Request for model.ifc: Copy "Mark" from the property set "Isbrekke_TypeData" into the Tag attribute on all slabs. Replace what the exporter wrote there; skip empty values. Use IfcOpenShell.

First a look at what the model holds.

```python
import ifcopenshell
import ifcopenshell.util.element

model = ifcopenshell.open("model.ifc")
print(model.schema)
slabs = model.by_type("IfcSlab")
print(len(slabs), "slabs")
for e in slabs[:8]:
    source = ifcopenshell.util.element.get_pset(e, "Isbrekke_TypeData", "Mark")
    target = e.Tag
    print(e.id(), repr(source), repr(target), sep=" | ")
```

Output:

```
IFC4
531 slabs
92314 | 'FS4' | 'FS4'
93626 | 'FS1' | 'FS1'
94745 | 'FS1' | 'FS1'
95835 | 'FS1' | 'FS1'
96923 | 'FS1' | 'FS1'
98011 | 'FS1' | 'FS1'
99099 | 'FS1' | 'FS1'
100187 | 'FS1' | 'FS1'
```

```python
import ifcopenshell
import ifcopenshell.util.element

model = ifcopenshell.open("model.ifc")

count = 0
for e in model.by_type("IfcSlab"):
    value = ifcopenshell.util.element.get_pset(e, "Isbrekke_TypeData", "Mark")
    current = e.Tag
    if not value or not value.strip() or current == value:
        continue
    e.Tag = value
    count += 1

print(count, "slabs updated")

model.write("model_edited.ifc")
```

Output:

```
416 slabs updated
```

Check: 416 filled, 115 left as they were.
